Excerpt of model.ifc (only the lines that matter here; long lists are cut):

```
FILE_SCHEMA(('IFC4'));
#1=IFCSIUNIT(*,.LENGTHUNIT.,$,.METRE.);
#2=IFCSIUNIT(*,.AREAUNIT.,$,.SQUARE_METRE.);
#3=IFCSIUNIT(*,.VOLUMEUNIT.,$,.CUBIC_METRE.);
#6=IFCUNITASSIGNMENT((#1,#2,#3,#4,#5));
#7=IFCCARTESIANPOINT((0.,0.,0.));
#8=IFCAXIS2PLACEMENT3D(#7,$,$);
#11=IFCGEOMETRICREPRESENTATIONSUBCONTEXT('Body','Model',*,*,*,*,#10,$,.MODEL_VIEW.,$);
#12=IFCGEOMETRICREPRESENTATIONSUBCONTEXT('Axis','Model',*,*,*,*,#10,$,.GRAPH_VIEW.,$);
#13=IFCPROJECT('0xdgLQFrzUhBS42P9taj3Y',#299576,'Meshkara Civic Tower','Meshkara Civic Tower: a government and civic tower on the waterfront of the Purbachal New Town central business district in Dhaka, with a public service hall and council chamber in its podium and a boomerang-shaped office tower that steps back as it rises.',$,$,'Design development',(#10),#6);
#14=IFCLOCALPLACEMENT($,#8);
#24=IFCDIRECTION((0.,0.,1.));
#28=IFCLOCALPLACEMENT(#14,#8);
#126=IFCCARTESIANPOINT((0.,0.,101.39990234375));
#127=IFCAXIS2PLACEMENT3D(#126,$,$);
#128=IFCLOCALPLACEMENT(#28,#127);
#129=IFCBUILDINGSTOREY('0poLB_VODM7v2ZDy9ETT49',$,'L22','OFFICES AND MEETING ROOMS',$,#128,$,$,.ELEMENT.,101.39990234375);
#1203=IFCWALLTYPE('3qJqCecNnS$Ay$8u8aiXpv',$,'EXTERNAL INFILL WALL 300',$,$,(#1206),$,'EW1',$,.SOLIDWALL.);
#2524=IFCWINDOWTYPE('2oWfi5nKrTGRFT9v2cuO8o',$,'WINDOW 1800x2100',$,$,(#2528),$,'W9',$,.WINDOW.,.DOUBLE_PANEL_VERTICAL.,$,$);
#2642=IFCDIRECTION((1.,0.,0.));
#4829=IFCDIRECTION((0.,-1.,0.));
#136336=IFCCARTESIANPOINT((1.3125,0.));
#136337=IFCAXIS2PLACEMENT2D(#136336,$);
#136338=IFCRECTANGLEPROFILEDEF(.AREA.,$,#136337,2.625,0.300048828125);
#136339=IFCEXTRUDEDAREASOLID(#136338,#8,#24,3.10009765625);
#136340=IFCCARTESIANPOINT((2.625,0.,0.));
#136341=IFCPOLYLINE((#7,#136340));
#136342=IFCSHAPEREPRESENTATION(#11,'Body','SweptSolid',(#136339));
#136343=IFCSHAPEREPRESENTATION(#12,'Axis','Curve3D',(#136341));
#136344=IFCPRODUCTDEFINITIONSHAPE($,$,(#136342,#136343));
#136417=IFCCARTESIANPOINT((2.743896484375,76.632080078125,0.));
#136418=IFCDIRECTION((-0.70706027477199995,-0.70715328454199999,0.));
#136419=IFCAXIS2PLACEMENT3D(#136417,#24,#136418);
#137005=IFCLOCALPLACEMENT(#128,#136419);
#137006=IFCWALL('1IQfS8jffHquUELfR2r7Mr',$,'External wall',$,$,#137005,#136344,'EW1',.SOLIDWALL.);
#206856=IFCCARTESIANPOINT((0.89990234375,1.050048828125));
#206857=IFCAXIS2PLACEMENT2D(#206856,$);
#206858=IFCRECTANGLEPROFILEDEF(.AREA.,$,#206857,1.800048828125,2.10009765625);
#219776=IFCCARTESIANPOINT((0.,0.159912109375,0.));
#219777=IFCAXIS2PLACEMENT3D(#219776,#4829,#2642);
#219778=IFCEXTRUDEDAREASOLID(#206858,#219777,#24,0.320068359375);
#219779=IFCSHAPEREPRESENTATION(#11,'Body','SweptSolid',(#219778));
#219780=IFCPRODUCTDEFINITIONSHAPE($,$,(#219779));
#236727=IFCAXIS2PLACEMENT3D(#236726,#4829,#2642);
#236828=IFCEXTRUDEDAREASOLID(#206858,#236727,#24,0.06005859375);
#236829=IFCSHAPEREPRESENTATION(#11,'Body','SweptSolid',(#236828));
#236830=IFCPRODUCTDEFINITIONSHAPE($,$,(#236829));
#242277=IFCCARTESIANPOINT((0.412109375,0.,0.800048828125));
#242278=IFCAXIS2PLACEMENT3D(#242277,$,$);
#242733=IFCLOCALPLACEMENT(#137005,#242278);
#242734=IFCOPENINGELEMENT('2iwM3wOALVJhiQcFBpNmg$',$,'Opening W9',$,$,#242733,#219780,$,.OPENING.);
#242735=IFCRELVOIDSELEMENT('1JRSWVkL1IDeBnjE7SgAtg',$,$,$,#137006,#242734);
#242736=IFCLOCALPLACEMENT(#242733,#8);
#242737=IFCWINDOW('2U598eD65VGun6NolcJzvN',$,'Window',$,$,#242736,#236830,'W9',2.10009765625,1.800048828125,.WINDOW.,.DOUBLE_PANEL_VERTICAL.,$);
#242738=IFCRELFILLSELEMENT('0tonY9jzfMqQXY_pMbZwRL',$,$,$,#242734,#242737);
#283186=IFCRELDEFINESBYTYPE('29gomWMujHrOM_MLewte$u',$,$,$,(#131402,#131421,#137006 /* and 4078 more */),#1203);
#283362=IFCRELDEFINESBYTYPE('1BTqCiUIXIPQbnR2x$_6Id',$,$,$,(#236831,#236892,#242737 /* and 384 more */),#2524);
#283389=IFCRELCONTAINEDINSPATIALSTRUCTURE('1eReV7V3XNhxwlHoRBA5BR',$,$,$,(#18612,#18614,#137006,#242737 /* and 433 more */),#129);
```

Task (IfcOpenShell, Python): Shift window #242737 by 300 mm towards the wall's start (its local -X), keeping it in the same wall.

```python
import ifcopenshell
import ifcopenshell.api.geometry
import ifcopenshell.util.placement
import ifcopenshell.util.unit

model = ifcopenshell.open("model.ifc")
unit_scale = ifcopenshell.util.unit.calculate_unit_scale(model)

window = model.by_guid("2U598eD65VGun6NolcJzvN")
opening = window.FillsVoids[0].RelatingOpeningElement
wall = opening.VoidsElements[0].RelatingBuildingElement

wall_matrix = ifcopenshell.util.placement.get_local_placement(wall.ObjectPlacement)
shift = wall_matrix[:3, 0] * -0.3 / unit_scale
before = ifcopenshell.util.placement.get_local_placement(window.ObjectPlacement)[:3, 3].copy()

# The window is placed relative to its opening, so it follows when the opening moves.
matrix = ifcopenshell.util.placement.get_local_placement(opening.ObjectPlacement)
matrix[:3, 3] += shift
ifcopenshell.api.geometry.edit_object_placement(
    model, product=opening, matrix=matrix, is_si=False, should_transform_children=True
)

after = ifcopenshell.util.placement.get_local_placement(window.ObjectPlacement)[:3, 3]
print("window moved by", (after - before).round(3) + 0.0)

model.write("model_v2.ifc")
```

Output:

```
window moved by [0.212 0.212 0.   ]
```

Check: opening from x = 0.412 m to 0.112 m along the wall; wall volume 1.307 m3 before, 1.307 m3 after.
